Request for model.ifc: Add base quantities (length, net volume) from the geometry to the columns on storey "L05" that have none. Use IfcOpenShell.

First a look at what the model holds.

```python
import ifcopenshell
import ifcopenshell.util.element
import ifcopenshell.util.unit

model = ifcopenshell.open("model.ifc")
print(model.schema)
for unit_type in ("LENGTHUNIT", "AREAUNIT", "VOLUMEUNIT"):
    print(unit_type, ifcopenshell.util.unit.calculate_unit_scale(model, unit_type))
storey = next(s for s in model.by_type("IfcBuildingStorey") if s.Name == "L05")
columns = [e for e in ifcopenshell.util.element.get_decomposition(storey) if e.is_a("IfcColumn")]
for e in sorted(columns, key=lambda e: e.id()):
    print(e.id(), e.is_a(), e.Name, list(ifcopenshell.util.element.get_psets(e, qtos_only=True)), sep=" | ")
```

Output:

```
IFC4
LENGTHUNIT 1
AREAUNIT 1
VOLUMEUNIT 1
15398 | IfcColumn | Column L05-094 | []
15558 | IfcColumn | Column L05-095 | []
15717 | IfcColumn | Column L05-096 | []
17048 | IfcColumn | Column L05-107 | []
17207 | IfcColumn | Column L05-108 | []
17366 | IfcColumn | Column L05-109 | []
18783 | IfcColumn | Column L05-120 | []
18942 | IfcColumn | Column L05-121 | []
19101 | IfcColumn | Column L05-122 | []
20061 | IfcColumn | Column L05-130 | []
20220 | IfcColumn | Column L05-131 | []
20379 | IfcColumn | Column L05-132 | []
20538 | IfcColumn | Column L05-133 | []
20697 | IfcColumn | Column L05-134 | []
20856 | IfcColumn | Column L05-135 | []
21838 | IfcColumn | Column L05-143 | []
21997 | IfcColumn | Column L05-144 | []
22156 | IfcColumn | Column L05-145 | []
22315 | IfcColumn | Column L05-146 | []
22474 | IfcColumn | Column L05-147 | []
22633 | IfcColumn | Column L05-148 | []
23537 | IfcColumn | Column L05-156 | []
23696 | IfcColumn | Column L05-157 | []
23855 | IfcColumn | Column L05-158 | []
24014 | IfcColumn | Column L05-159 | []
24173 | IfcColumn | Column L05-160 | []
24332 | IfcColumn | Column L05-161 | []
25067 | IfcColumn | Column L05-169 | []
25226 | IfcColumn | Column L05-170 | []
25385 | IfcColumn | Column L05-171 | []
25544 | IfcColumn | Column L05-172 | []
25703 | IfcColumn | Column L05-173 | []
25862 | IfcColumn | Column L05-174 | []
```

```python
import ifcopenshell
import ifcopenshell.api.pset
import ifcopenshell.geom
import ifcopenshell.util.element
import ifcopenshell.util.shape
import ifcopenshell.util.unit

model = ifcopenshell.open("model.ifc")
unit_scale = ifcopenshell.util.unit.calculate_unit_scale(model)
volume_scale = ifcopenshell.util.unit.calculate_unit_scale(model, "VOLUMEUNIT")
settings = ifcopenshell.geom.settings()

storey = next(s for s in model.by_type("IfcBuildingStorey") if s.Name == "L05")
columns = [e for e in ifcopenshell.util.element.get_decomposition(storey) if e.is_a("IfcColumn")]

for e in sorted(columns, key=lambda e: e.id()):
    if ifcopenshell.util.element.get_psets(e, qtos_only=True, should_inherit=False):
        continue
    # Geometry comes back in metres, in the element's own axes.
    shape = ifcopenshell.geom.create_shape(settings, e)
    values = {
        "Length": ifcopenshell.util.shape.get_z(shape.geometry) / unit_scale,
        "NetVolume": ifcopenshell.util.shape.get_volume(shape.geometry) / volume_scale,
    }
    qto = ifcopenshell.api.pset.add_qto(model, product=e, name="Qto_ColumnBaseQuantities")
    ifcopenshell.api.pset.edit_qto(model, qto=qto, properties=values)
    print(e.id(), {k: round(v, 3) for k, v in values.items()})

model.write("model_updated.ifc")
```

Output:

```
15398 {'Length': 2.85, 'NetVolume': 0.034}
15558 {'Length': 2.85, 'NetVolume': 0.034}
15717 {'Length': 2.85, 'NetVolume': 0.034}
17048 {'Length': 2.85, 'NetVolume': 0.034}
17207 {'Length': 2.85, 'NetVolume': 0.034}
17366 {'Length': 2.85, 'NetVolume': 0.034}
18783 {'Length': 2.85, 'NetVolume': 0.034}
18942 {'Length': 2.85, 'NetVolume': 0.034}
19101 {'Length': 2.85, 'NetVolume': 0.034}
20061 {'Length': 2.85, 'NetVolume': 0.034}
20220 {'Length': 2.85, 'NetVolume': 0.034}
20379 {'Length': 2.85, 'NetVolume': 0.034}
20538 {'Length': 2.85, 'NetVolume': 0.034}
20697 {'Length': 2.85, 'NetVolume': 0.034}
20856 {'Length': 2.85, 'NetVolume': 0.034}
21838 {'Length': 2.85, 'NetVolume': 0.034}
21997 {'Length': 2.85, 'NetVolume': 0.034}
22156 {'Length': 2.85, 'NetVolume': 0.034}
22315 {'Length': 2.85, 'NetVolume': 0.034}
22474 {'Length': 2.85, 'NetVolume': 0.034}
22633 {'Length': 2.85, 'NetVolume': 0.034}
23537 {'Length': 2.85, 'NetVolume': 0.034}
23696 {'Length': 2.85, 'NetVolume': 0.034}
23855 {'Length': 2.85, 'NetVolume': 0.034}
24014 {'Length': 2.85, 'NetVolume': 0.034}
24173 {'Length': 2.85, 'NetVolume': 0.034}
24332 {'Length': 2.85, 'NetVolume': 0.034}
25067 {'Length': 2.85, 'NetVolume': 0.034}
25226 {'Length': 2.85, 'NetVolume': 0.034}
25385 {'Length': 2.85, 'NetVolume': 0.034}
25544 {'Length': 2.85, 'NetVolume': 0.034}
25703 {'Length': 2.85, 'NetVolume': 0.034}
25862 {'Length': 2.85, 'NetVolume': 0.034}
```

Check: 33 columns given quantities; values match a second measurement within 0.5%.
